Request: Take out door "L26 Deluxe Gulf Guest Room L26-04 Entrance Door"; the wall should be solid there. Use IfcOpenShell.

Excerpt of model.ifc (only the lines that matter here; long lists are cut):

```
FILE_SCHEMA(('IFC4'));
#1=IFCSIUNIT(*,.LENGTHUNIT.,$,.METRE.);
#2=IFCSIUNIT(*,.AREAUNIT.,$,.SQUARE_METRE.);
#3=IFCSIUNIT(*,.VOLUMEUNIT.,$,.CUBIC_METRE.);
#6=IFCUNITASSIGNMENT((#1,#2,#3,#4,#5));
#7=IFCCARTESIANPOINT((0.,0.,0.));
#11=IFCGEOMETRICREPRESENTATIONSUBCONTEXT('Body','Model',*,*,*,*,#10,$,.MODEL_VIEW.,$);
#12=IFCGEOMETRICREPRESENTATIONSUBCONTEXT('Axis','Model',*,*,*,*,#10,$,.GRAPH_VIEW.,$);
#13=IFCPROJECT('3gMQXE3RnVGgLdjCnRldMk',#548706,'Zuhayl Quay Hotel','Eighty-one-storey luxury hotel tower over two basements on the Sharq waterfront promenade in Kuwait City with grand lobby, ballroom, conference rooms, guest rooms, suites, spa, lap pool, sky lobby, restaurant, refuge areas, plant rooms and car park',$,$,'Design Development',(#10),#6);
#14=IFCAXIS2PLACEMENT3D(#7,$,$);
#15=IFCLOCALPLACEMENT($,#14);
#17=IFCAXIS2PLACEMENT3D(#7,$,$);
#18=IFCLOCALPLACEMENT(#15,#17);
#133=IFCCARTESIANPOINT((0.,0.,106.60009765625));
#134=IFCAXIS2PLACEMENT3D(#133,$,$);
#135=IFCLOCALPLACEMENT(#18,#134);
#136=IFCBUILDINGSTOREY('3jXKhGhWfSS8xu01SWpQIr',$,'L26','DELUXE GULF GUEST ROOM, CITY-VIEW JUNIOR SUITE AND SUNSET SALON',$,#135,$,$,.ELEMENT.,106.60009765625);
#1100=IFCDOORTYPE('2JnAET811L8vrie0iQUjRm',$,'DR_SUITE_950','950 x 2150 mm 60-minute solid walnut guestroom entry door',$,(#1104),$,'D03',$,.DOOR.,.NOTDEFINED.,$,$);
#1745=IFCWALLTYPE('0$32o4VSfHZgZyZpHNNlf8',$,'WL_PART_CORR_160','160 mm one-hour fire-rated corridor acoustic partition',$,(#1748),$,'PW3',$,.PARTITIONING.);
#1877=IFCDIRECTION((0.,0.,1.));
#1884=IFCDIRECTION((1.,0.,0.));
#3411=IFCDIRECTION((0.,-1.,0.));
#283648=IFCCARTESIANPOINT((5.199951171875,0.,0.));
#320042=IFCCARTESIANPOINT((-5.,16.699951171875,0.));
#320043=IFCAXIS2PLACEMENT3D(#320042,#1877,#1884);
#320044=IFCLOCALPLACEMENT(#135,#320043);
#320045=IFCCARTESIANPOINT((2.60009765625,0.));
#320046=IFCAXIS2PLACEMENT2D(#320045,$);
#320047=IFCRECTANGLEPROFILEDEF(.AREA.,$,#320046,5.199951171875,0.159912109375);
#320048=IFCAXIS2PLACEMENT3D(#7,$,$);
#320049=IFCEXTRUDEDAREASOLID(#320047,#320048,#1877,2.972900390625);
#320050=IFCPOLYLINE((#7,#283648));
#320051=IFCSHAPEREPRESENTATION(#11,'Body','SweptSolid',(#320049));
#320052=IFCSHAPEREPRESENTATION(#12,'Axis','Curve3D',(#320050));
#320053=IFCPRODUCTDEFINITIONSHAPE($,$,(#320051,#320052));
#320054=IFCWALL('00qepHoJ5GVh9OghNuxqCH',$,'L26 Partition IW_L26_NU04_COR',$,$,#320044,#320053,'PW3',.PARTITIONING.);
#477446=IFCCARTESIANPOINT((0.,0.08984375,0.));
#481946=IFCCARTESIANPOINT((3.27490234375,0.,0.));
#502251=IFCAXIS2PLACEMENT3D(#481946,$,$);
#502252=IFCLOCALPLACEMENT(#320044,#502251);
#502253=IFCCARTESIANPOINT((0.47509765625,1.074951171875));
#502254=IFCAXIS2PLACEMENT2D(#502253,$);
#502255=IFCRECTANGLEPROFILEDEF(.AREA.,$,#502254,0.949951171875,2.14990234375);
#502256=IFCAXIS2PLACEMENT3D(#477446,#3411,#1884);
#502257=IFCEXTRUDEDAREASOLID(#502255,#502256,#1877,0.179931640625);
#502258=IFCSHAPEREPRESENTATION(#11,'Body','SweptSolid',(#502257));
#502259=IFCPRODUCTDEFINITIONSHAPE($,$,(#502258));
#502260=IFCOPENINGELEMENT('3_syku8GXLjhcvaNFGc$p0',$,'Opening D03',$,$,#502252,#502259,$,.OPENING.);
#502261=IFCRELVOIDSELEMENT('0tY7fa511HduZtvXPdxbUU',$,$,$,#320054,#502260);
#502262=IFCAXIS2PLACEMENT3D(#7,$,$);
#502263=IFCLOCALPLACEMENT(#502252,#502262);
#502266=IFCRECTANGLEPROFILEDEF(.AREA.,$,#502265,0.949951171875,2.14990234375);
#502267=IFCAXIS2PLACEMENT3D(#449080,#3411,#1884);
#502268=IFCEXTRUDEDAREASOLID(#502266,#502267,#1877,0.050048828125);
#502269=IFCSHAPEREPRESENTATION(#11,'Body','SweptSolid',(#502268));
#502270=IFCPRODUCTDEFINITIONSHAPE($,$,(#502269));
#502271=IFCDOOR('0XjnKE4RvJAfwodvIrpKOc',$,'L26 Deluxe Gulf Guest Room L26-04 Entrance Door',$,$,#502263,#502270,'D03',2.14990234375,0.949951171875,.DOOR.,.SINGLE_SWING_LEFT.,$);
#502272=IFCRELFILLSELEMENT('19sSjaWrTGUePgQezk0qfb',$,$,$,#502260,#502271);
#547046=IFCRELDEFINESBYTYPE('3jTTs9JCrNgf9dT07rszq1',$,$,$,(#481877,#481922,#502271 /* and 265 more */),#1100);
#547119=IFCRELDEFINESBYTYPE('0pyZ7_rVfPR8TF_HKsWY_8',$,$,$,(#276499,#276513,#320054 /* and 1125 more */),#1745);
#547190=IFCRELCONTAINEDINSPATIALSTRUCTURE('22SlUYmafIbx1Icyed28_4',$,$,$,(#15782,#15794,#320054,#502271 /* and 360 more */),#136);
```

```python
import ifcopenshell
import ifcopenshell.api.feature
import ifcopenshell.api.root
import ifcopenshell.geom
import ifcopenshell.util.shape

model = ifcopenshell.open("model.ifc")
settings = ifcopenshell.geom.settings()


def volume(element):
    """Net volume in cubic metres, openings subtracted."""
    shape = ifcopenshell.geom.create_shape(settings, element)
    return ifcopenshell.util.shape.get_volume(shape.geometry)


door = model.by_guid("0XjnKE4RvJAfwodvIrpKOc")
opening = door.FillsVoids[0].RelatingOpeningElement
wall = opening.VoidsElements[0].RelatingBuildingElement
before = volume(wall)

ifcopenshell.api.root.remove_product(model, product=door)
ifcopenshell.api.feature.remove_feature(model, feature=opening)

after = volume(wall)

print(f"wall volume {before:.3f} -> {after:.3f} m3")

model.write("model_updated.ifc")
```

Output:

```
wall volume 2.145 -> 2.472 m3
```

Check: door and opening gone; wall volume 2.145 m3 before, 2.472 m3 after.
